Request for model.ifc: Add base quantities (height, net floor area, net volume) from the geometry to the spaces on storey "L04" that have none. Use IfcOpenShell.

First a look at what the model holds.

```python
import ifcopenshell
import ifcopenshell.util.element
import ifcopenshell.util.unit

model = ifcopenshell.open("model.ifc")
print(model.schema)
for unit_type in ("LENGTHUNIT", "AREAUNIT", "VOLUMEUNIT"):
    print(unit_type, ifcopenshell.util.unit.calculate_unit_scale(model, unit_type))
storey = next(s for s in model.by_type("IfcBuildingStorey") if s.Name == "L04")
spaces = [e for e in ifcopenshell.util.element.get_decomposition(storey) if e.is_a("IfcSpace")]
for e in sorted(spaces, key=lambda e: e.id()):
    print(e.id(), e.is_a(), e.Name, list(ifcopenshell.util.element.get_psets(e, qtos_only=True)), sep=" | ")
```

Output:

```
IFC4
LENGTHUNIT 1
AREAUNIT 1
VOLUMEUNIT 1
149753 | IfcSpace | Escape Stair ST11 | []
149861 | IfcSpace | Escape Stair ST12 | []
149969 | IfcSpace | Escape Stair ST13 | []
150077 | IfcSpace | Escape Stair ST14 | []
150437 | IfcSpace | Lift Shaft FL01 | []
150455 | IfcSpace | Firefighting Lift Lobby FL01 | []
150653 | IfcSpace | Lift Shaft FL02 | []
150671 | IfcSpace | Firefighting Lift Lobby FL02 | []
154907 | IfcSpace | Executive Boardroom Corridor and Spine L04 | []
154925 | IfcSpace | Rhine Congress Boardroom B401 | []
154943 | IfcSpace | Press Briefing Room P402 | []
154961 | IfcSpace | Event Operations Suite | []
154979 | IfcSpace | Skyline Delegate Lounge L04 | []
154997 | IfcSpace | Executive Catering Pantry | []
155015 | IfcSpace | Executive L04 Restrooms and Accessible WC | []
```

```python
import ifcopenshell
import ifcopenshell.api.pset
import ifcopenshell.geom
import ifcopenshell.util.element
import ifcopenshell.util.shape
import ifcopenshell.util.unit

model = ifcopenshell.open("model.ifc")
unit_scale = ifcopenshell.util.unit.calculate_unit_scale(model)
area_scale = ifcopenshell.util.unit.calculate_unit_scale(model, "AREAUNIT")
volume_scale = ifcopenshell.util.unit.calculate_unit_scale(model, "VOLUMEUNIT")
settings = ifcopenshell.geom.settings()

storey = next(s for s in model.by_type("IfcBuildingStorey") if s.Name == "L04")
spaces = [e for e in ifcopenshell.util.element.get_decomposition(storey) if e.is_a("IfcSpace")]

for e in sorted(spaces, key=lambda e: e.id()):
    if ifcopenshell.util.element.get_psets(e, qtos_only=True, should_inherit=False):
        continue
    # Geometry comes back in metres, in the element's own axes.
    shape = ifcopenshell.geom.create_shape(settings, e)
    values = {
        "Height": ifcopenshell.util.shape.get_z(shape.geometry) / unit_scale,
        "NetFloorArea": ifcopenshell.util.shape.get_footprint_area(shape.geometry) / area_scale,
        "NetVolume": ifcopenshell.util.shape.get_volume(shape.geometry) / volume_scale,
    }
    qto = ifcopenshell.api.pset.add_qto(model, product=e, name="Qto_SpaceBaseQuantities")
    ifcopenshell.api.pset.edit_qto(model, qto=qto, properties=values)
    print(e.id(), {k: round(v, 3) for k, v in values.items()})

model.write("model_v2.ifc")
```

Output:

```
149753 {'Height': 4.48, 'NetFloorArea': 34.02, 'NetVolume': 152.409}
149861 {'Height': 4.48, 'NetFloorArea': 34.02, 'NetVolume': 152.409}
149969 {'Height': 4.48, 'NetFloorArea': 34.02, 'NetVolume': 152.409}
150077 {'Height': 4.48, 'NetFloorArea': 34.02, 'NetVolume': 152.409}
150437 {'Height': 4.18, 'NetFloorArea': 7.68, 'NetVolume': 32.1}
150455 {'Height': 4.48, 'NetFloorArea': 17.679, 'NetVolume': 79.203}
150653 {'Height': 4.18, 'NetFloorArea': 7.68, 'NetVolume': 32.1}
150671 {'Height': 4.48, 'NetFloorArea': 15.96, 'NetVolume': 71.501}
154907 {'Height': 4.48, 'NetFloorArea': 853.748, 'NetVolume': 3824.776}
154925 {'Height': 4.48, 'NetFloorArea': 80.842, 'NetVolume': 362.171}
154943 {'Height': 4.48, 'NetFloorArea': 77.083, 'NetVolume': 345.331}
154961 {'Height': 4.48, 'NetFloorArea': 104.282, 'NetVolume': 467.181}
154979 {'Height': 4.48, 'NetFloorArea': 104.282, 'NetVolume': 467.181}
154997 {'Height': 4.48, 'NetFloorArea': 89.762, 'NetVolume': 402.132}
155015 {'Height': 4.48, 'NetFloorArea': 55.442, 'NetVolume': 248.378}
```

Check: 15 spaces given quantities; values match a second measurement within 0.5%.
